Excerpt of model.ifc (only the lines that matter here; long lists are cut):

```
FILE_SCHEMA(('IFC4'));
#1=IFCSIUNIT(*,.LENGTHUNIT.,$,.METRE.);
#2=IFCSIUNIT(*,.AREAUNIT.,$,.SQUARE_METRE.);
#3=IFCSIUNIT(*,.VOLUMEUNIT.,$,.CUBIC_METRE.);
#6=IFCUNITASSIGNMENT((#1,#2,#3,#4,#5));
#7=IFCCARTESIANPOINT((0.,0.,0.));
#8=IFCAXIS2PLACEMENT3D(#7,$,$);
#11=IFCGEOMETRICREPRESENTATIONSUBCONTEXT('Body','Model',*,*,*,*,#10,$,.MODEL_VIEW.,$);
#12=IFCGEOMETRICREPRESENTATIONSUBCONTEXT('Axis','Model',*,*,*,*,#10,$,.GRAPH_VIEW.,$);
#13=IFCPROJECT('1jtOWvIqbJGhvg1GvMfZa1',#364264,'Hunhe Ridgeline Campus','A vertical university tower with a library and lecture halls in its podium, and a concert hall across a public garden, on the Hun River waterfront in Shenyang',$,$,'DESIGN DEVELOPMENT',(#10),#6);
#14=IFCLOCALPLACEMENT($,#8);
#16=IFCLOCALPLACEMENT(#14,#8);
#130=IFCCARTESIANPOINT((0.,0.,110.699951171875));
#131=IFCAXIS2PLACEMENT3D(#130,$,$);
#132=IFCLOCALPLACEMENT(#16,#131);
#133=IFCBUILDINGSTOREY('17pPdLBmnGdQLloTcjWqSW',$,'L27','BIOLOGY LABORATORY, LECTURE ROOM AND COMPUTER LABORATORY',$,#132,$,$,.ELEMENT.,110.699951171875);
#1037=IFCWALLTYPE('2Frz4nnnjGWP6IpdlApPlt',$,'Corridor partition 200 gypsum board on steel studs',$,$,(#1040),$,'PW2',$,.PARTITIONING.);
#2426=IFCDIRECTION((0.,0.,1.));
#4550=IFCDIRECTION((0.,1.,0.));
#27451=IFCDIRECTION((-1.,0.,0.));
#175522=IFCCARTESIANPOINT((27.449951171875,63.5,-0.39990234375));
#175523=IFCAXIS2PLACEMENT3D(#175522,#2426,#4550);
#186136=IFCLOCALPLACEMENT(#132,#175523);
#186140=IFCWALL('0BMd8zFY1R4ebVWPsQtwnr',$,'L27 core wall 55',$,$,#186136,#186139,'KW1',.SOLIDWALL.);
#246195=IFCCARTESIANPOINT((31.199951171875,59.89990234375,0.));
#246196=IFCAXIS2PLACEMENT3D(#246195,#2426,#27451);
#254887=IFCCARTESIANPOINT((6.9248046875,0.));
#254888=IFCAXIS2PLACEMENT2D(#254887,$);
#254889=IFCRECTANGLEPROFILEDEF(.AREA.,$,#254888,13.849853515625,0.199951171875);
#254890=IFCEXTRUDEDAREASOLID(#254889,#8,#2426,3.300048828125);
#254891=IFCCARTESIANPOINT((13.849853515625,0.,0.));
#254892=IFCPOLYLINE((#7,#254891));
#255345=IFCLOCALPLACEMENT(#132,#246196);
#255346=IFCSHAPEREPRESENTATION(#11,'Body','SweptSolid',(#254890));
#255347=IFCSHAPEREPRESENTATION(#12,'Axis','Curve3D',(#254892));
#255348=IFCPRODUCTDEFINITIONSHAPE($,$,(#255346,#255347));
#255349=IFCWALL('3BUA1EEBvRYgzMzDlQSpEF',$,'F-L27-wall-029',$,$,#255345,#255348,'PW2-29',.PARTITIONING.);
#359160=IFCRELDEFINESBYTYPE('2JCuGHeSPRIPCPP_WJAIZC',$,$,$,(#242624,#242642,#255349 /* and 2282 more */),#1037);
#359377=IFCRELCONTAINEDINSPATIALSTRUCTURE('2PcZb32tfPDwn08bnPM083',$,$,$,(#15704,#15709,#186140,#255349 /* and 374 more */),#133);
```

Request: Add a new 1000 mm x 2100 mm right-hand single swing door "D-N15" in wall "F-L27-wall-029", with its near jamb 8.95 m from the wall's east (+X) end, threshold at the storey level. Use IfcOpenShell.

```python
import numpy as np
import ifcopenshell
import ifcopenshell.api.feature
import ifcopenshell.api.geometry
import ifcopenshell.api.root
import ifcopenshell.api.spatial
import ifcopenshell.geom
import ifcopenshell.util.element
import ifcopenshell.util.placement
import ifcopenshell.util.representation
import ifcopenshell.util.shape
import ifcopenshell.util.unit

model = ifcopenshell.open("model.ifc")
unit_scale = ifcopenshell.util.unit.calculate_unit_scale(model)
settings = ifcopenshell.geom.settings()


def volume(element):
    """Net volume in cubic metres, openings subtracted."""
    shape = ifcopenshell.geom.create_shape(settings, element)
    return ifcopenshell.util.shape.get_volume(shape.geometry)


wall = model.by_guid("3BUA1EEBvRYgzMzDlQSpEF")
storey = ifcopenshell.util.element.get_container(wall, ifc_class="IfcBuildingStorey")
context = ifcopenshell.util.representation.get_context(model, "Model", "Body", "MODEL_VIEW")
before = volume(wall)

width, height, from_end, sill = 1, 2.1, 8.95, 0.0  # metres

# The wall runs along its own X axis, and the end named is its -X end.
wall_shape = ifcopenshell.geom.create_shape(settings, wall)
x, y, z = ifcopenshell.util.shape.get_vertices(wall_shape.geometry).T
start = x.min() + from_end
face, thickness = float(y.min()), float(y.max() - y.min())
wall_matrix = ifcopenshell.util.placement.get_local_placement(wall.ObjectPlacement)
level = ifcopenshell.util.placement.get_local_placement(storey.ObjectPlacement)[2, 3]


def in_wall(x, y):
    """Placement at x, y metres in the wall's axes, at sill height."""
    matrix = wall_matrix.copy()
    matrix[:, 3] = wall_matrix @ np.array([x / unit_scale, y / unit_scale, 0.0, 1.0])
    matrix[2, 3] = level + sill / unit_scale
    return matrix


# Opening: a box that overshoots both wall faces by 50 mm.
opening = ifcopenshell.api.root.create_entity(model, ifc_class="IfcOpeningElement", predefined_type="OPENING")
box = ifcopenshell.api.geometry.add_wall_representation(
    model, context=context, length=width, height=height, thickness=thickness + 0.1
)
ifcopenshell.api.geometry.assign_representation(model, product=opening, representation=box)
ifcopenshell.api.geometry.edit_object_placement(model, product=opening, matrix=in_wall(start, face - 0.05), is_si=False)
ifcopenshell.api.feature.add_feature(model, feature=opening, element=wall)

door = ifcopenshell.api.root.create_entity(model, ifc_class="IfcDoor", name="D-N15", predefined_type="DOOR")
door.OverallWidth, door.OverallHeight = width / unit_scale, height / unit_scale
door.OperationType = "SINGLE_SWING_RIGHT"
body = ifcopenshell.api.geometry.add_door_representation(
    model,
    context=context,
    overall_width=door.OverallWidth,
    overall_height=door.OverallHeight,
    operation_type="SINGLE_SWING_RIGHT",
    lining_properties={"LiningDepth": thickness / unit_scale, "ThresholdDepth": thickness / unit_scale},
)
ifcopenshell.api.geometry.assign_representation(model, product=door, representation=body)
ifcopenshell.api.spatial.assign_container(model, products=[door], relating_structure=storey)
ifcopenshell.api.feature.add_filling(model, opening=opening, element=door)

# The lining spans the wall, so the door starts at the wall face.
ifcopenshell.api.geometry.edit_object_placement(model, product=door, matrix=in_wall(start, face), is_si=False)

after = volume(wall)

print(f"wall volume {before:.3f} -> {after:.3f} m3")

model.write("model_rev.ifc")
```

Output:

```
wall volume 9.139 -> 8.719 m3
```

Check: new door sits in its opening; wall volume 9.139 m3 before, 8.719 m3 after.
